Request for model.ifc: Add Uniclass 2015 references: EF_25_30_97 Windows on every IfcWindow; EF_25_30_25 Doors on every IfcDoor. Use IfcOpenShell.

First a look at what the model holds.

```python
import ifcopenshell

model = ifcopenshell.open("model.ifc")
print(model.schema)
print("classifications:", [c.Name for c in model.by_type("IfcClassification")])
for ifc_class in ("IfcDoor", "IfcRoof", "IfcStair", "IfcWall", "IfcWindow"):
    print(ifc_class, len(model.by_type(ifc_class)))
```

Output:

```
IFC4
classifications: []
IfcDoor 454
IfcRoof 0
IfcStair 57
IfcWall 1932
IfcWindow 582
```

```python
import ifcopenshell
import ifcopenshell.api.classification

model = ifcopenshell.open("model.ifc")

system = ifcopenshell.api.classification.add_classification(model, classification="Uniclass 2015")

codes = {
    "IfcWindow": ("EF_25_30_97", "Windows"),
    "IfcDoor": ("EF_25_30_25", "Doors"),
}
for ifc_class, (code, name) in codes.items():
    products = model.by_type(ifc_class)
    ifcopenshell.api.classification.add_reference(
        model, products=products, classification=system, identification=code, name=name
    )
    print(code, len(products))

model.write("model_edited.ifc")
```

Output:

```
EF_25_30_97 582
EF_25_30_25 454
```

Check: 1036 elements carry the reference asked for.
